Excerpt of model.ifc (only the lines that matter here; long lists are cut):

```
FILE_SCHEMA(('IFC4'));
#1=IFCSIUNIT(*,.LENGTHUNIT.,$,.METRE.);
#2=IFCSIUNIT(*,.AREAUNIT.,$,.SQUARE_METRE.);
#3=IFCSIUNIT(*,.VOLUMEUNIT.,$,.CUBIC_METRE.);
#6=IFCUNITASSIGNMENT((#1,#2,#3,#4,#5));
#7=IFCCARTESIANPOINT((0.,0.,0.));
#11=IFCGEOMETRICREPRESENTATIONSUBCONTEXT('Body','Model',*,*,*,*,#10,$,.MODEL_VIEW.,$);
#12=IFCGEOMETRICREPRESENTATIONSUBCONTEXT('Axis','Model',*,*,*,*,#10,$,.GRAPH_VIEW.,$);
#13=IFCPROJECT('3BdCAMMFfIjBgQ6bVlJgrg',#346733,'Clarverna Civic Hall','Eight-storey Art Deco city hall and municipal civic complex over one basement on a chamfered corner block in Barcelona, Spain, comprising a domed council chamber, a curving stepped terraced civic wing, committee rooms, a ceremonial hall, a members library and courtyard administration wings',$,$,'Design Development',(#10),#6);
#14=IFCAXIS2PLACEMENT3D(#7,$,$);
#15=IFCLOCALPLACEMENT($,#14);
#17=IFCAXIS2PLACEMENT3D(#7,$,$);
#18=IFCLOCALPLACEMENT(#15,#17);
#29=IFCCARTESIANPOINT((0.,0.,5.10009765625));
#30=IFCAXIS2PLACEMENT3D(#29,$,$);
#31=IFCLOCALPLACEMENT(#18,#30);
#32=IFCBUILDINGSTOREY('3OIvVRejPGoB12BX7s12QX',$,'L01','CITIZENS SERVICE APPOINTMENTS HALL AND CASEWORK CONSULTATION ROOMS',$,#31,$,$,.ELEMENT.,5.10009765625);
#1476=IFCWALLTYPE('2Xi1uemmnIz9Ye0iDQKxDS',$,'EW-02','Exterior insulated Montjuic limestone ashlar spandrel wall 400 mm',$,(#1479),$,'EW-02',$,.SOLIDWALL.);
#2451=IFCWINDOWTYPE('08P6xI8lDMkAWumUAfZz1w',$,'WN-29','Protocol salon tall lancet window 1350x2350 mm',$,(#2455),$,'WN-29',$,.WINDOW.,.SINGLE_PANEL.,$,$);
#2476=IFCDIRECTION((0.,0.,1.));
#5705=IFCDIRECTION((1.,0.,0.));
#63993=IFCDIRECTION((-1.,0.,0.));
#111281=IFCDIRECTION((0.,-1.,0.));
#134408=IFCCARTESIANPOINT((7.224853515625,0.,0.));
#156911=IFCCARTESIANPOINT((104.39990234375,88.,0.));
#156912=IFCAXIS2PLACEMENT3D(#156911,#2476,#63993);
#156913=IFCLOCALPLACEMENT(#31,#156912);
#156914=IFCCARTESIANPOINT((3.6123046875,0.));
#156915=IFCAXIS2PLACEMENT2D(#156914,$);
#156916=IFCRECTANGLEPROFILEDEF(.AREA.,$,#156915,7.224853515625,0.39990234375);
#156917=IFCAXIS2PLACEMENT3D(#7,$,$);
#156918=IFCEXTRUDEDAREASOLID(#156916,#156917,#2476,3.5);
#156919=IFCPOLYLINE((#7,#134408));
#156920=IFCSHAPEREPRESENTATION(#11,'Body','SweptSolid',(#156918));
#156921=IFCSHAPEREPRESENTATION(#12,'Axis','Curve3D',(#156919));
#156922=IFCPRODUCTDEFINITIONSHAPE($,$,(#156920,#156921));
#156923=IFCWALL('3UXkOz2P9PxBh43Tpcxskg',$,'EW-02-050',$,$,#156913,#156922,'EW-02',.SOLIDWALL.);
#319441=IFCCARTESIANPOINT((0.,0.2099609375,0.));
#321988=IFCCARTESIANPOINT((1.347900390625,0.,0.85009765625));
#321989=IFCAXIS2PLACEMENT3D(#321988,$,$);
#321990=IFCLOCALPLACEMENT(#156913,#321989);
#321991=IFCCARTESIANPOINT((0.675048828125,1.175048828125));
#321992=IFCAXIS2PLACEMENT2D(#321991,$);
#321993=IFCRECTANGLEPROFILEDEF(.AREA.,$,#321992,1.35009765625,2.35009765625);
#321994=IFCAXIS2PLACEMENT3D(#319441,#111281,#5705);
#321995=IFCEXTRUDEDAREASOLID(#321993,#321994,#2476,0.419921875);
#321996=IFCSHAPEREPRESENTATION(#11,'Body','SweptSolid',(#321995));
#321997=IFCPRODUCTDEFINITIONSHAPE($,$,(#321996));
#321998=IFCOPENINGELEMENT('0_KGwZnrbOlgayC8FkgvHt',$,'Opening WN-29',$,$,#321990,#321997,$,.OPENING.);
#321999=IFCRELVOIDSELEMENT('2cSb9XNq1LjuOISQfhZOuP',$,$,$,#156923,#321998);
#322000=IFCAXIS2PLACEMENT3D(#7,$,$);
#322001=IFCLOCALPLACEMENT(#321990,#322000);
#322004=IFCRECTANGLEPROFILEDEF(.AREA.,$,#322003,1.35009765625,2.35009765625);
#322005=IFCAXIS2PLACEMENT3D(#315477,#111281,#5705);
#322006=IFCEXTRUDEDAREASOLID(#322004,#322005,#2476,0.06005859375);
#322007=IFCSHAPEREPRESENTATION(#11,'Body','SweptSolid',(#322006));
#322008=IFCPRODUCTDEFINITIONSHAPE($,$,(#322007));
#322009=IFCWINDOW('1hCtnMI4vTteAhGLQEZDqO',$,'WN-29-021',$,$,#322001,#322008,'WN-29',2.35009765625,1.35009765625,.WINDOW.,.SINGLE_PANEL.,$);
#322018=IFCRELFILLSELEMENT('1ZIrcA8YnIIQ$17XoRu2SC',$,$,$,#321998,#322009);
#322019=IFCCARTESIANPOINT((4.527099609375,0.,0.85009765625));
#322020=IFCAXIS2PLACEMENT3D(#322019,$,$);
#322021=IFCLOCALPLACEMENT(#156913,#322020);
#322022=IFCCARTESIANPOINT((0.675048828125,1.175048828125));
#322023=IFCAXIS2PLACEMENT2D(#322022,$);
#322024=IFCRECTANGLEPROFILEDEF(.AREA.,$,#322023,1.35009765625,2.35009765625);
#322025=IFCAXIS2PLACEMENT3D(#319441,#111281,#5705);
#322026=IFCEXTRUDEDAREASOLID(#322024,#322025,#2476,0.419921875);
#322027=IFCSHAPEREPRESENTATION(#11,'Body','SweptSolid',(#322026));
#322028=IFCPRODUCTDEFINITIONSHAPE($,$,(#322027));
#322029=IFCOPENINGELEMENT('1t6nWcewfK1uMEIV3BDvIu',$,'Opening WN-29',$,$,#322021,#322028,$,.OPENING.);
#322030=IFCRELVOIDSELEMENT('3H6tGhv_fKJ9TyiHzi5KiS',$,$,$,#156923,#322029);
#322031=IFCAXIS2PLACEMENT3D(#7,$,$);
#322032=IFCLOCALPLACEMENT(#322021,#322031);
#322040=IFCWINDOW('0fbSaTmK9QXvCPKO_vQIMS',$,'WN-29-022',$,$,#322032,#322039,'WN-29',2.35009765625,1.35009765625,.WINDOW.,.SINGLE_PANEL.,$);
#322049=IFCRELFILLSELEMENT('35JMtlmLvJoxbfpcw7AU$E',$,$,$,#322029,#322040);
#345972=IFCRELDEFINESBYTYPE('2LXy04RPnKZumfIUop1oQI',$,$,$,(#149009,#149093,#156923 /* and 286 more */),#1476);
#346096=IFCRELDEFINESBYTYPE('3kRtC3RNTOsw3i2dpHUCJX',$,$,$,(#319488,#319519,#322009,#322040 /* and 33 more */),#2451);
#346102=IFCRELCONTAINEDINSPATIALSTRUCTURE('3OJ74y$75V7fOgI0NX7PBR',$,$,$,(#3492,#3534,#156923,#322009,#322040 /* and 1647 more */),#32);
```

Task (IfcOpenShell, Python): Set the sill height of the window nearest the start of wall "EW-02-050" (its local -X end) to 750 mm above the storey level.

```python
import numpy as np
import ifcopenshell
import ifcopenshell.api.geometry
import ifcopenshell.geom
import ifcopenshell.util.element
import ifcopenshell.util.placement
import ifcopenshell.util.shape
import ifcopenshell.util.unit

model = ifcopenshell.open("model.ifc")
unit_scale = ifcopenshell.util.unit.calculate_unit_scale(model)

window = model.by_guid("1hCtnMI4vTteAhGLQEZDqO")
opening = window.FillsVoids[0].RelatingOpeningElement
storey = ifcopenshell.util.element.get_container(window, ifc_class="IfcBuildingStorey")
level = ifcopenshell.util.placement.get_local_placement(storey.ObjectPlacement)[2, 3]

# The opening's origin need not be at the sill, so measure its lowest point.
shape = ifcopenshell.geom.create_shape(ifcopenshell.geom.settings(), opening)
bottom = ifcopenshell.util.shape.get_shape_bottom_elevation(shape, shape.geometry) / unit_scale
dz = level + 0.75 / unit_scale - bottom

shift = np.array([0.0, 0.0, dz])
# The window is placed relative to its opening, so it follows when the opening moves.
matrix = ifcopenshell.util.placement.get_local_placement(opening.ObjectPlacement)
matrix[:3, 3] += shift
ifcopenshell.api.geometry.edit_object_placement(
    model, product=opening, matrix=matrix, is_si=False, should_transform_children=True
)

print(f"moved by {dz * unit_scale:+.3f} m")

model.write("model_edited.ifc")
```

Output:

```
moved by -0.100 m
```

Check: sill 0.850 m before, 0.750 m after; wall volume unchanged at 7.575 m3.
